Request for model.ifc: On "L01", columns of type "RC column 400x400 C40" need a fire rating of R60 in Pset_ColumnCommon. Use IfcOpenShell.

First a look at what the model holds.

```python
import ifcopenshell
import ifcopenshell.util.element

model = ifcopenshell.open("model.ifc")
print(model.schema)
storey = next(s for s in model.by_type("IfcBuildingStorey") if s.Name == "L01")
columns = [e for e in ifcopenshell.util.element.get_decomposition(storey) if e.is_a("IfcColumn")]
seen = {}
for e in columns:
    element_type = ifcopenshell.util.element.get_type(e)
    key = (element_type.Name if element_type != e and element_type else None, ifcopenshell.util.element.get_pset(e, "Pset_ColumnCommon", "FireRating"))
    seen[key] = seen.get(key, 0) + 1
for (name, value), count in sorted(seen.items(), key=str):
    print(count, "x", name, "|", value)
```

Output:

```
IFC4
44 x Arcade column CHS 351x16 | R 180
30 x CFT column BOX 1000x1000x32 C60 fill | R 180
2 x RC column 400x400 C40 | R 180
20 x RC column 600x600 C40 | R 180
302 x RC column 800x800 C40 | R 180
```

```python
import ifcopenshell
import ifcopenshell.api.pset
import ifcopenshell.util.element

model = ifcopenshell.open("model.ifc")

storey = next(s for s in model.by_type("IfcBuildingStorey") if s.Name == "L01")
columns = [e for e in ifcopenshell.util.element.get_decomposition(storey) if e.is_a("IfcColumn")]

count = 0
for e in columns:
    element_type = ifcopenshell.util.element.get_type(e)
    if element_type in (None, e) or element_type.Name != "RC column 400x400 C40":
        continue
    # add_pset returns the element's existing set when there is one.
    pset = ifcopenshell.api.pset.add_pset(model, product=e, name="Pset_ColumnCommon")
    ifcopenshell.api.pset.edit_pset(model, pset=pset, properties={"FireRating": "R60"})
    count += 1

print(count, "columns updated")

model.write("model-out.ifc")
```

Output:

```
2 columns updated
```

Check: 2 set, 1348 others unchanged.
